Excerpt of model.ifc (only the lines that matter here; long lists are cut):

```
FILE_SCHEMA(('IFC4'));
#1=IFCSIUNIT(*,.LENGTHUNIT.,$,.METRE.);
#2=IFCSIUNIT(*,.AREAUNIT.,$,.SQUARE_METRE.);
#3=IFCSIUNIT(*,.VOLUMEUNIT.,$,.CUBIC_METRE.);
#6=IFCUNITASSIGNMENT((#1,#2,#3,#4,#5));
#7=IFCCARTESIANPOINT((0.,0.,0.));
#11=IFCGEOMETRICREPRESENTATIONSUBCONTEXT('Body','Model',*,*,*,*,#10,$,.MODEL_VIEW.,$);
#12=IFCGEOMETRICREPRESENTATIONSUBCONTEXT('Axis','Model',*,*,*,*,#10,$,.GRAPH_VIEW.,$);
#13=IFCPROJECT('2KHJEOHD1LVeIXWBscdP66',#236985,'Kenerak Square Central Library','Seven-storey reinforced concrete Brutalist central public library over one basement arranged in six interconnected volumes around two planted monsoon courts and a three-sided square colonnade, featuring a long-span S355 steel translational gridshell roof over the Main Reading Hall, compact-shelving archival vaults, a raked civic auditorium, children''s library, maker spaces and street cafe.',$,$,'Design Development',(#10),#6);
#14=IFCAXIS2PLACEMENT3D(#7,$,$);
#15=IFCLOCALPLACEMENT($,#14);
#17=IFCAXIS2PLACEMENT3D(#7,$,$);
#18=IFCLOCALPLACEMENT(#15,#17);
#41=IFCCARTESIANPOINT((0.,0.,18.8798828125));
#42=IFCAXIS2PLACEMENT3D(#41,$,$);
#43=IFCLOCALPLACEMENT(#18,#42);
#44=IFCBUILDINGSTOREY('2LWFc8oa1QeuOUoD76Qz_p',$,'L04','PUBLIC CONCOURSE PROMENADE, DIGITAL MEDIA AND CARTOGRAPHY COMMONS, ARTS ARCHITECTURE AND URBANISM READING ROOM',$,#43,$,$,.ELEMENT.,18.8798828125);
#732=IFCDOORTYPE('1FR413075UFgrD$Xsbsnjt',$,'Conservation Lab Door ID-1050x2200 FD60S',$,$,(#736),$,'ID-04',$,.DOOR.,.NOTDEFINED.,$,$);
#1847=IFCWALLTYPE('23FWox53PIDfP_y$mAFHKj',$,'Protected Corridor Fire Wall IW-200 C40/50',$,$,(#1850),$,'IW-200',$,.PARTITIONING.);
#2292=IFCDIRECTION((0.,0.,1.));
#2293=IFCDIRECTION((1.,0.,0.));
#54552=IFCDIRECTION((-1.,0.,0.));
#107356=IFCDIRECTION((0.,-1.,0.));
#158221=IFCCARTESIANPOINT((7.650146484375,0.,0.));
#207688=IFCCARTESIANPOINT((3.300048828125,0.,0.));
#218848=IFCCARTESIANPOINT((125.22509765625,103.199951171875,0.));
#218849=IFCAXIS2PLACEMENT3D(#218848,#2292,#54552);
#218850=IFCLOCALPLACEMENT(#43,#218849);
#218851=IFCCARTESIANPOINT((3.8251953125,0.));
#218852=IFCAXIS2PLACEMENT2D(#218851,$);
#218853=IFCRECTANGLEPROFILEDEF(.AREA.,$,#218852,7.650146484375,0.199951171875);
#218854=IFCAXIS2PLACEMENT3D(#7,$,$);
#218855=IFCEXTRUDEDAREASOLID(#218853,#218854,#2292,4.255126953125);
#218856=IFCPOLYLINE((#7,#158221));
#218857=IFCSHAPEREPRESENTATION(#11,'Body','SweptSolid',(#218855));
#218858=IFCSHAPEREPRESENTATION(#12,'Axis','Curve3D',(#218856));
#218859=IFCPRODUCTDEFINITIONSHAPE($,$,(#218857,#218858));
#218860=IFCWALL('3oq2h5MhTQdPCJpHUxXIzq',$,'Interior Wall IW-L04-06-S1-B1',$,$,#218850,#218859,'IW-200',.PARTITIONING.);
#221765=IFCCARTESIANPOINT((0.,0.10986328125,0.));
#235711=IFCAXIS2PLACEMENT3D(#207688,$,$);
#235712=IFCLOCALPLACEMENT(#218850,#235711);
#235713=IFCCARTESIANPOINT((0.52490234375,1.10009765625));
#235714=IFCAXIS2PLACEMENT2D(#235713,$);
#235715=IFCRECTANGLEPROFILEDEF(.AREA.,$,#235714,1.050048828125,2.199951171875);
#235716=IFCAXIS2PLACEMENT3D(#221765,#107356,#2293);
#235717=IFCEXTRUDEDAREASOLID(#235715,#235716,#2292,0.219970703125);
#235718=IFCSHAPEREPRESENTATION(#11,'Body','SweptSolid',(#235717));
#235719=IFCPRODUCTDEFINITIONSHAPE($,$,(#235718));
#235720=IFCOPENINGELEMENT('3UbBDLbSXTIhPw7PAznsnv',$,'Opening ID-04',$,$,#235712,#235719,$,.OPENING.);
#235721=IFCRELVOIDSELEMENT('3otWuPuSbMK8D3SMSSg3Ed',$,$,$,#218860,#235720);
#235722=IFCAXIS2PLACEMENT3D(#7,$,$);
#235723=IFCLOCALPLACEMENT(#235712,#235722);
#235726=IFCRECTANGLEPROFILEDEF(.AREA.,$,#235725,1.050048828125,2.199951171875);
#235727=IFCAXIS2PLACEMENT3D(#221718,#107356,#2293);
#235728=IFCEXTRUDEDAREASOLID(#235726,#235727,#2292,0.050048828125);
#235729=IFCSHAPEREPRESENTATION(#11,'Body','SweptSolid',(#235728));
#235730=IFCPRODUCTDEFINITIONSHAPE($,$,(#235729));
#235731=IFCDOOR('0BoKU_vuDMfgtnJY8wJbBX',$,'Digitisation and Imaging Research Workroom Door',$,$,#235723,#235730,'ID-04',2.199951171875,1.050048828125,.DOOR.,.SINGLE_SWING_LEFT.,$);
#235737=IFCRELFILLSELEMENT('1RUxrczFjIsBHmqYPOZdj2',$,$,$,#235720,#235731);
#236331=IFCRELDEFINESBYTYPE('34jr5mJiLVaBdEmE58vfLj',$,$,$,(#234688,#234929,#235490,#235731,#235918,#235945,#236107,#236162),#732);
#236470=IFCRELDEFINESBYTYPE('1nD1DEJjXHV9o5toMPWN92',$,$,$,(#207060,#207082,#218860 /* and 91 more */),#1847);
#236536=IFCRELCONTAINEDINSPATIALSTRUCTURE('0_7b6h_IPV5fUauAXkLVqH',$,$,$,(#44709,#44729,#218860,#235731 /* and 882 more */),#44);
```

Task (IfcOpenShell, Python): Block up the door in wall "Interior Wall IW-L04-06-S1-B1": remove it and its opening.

```python
import ifcopenshell
import ifcopenshell.api.feature
import ifcopenshell.api.root
import ifcopenshell.geom
import ifcopenshell.util.shape

model = ifcopenshell.open("model.ifc")
settings = ifcopenshell.geom.settings()


def volume(element):
    """Net volume in cubic metres, openings subtracted."""
    shape = ifcopenshell.geom.create_shape(settings, element)
    return ifcopenshell.util.shape.get_volume(shape.geometry)


door = model.by_guid("0BoKU_vuDMfgtnJY8wJbBX")
opening = door.FillsVoids[0].RelatingOpeningElement
wall = opening.VoidsElements[0].RelatingBuildingElement
before = volume(wall)

ifcopenshell.api.root.remove_product(model, product=door)
ifcopenshell.api.feature.remove_feature(model, feature=opening)

after = volume(wall)

print(f"wall volume {before:.3f} -> {after:.3f} m3")

model.write("model_updated.ifc")
```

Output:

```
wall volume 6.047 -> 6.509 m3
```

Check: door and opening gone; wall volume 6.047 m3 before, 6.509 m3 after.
